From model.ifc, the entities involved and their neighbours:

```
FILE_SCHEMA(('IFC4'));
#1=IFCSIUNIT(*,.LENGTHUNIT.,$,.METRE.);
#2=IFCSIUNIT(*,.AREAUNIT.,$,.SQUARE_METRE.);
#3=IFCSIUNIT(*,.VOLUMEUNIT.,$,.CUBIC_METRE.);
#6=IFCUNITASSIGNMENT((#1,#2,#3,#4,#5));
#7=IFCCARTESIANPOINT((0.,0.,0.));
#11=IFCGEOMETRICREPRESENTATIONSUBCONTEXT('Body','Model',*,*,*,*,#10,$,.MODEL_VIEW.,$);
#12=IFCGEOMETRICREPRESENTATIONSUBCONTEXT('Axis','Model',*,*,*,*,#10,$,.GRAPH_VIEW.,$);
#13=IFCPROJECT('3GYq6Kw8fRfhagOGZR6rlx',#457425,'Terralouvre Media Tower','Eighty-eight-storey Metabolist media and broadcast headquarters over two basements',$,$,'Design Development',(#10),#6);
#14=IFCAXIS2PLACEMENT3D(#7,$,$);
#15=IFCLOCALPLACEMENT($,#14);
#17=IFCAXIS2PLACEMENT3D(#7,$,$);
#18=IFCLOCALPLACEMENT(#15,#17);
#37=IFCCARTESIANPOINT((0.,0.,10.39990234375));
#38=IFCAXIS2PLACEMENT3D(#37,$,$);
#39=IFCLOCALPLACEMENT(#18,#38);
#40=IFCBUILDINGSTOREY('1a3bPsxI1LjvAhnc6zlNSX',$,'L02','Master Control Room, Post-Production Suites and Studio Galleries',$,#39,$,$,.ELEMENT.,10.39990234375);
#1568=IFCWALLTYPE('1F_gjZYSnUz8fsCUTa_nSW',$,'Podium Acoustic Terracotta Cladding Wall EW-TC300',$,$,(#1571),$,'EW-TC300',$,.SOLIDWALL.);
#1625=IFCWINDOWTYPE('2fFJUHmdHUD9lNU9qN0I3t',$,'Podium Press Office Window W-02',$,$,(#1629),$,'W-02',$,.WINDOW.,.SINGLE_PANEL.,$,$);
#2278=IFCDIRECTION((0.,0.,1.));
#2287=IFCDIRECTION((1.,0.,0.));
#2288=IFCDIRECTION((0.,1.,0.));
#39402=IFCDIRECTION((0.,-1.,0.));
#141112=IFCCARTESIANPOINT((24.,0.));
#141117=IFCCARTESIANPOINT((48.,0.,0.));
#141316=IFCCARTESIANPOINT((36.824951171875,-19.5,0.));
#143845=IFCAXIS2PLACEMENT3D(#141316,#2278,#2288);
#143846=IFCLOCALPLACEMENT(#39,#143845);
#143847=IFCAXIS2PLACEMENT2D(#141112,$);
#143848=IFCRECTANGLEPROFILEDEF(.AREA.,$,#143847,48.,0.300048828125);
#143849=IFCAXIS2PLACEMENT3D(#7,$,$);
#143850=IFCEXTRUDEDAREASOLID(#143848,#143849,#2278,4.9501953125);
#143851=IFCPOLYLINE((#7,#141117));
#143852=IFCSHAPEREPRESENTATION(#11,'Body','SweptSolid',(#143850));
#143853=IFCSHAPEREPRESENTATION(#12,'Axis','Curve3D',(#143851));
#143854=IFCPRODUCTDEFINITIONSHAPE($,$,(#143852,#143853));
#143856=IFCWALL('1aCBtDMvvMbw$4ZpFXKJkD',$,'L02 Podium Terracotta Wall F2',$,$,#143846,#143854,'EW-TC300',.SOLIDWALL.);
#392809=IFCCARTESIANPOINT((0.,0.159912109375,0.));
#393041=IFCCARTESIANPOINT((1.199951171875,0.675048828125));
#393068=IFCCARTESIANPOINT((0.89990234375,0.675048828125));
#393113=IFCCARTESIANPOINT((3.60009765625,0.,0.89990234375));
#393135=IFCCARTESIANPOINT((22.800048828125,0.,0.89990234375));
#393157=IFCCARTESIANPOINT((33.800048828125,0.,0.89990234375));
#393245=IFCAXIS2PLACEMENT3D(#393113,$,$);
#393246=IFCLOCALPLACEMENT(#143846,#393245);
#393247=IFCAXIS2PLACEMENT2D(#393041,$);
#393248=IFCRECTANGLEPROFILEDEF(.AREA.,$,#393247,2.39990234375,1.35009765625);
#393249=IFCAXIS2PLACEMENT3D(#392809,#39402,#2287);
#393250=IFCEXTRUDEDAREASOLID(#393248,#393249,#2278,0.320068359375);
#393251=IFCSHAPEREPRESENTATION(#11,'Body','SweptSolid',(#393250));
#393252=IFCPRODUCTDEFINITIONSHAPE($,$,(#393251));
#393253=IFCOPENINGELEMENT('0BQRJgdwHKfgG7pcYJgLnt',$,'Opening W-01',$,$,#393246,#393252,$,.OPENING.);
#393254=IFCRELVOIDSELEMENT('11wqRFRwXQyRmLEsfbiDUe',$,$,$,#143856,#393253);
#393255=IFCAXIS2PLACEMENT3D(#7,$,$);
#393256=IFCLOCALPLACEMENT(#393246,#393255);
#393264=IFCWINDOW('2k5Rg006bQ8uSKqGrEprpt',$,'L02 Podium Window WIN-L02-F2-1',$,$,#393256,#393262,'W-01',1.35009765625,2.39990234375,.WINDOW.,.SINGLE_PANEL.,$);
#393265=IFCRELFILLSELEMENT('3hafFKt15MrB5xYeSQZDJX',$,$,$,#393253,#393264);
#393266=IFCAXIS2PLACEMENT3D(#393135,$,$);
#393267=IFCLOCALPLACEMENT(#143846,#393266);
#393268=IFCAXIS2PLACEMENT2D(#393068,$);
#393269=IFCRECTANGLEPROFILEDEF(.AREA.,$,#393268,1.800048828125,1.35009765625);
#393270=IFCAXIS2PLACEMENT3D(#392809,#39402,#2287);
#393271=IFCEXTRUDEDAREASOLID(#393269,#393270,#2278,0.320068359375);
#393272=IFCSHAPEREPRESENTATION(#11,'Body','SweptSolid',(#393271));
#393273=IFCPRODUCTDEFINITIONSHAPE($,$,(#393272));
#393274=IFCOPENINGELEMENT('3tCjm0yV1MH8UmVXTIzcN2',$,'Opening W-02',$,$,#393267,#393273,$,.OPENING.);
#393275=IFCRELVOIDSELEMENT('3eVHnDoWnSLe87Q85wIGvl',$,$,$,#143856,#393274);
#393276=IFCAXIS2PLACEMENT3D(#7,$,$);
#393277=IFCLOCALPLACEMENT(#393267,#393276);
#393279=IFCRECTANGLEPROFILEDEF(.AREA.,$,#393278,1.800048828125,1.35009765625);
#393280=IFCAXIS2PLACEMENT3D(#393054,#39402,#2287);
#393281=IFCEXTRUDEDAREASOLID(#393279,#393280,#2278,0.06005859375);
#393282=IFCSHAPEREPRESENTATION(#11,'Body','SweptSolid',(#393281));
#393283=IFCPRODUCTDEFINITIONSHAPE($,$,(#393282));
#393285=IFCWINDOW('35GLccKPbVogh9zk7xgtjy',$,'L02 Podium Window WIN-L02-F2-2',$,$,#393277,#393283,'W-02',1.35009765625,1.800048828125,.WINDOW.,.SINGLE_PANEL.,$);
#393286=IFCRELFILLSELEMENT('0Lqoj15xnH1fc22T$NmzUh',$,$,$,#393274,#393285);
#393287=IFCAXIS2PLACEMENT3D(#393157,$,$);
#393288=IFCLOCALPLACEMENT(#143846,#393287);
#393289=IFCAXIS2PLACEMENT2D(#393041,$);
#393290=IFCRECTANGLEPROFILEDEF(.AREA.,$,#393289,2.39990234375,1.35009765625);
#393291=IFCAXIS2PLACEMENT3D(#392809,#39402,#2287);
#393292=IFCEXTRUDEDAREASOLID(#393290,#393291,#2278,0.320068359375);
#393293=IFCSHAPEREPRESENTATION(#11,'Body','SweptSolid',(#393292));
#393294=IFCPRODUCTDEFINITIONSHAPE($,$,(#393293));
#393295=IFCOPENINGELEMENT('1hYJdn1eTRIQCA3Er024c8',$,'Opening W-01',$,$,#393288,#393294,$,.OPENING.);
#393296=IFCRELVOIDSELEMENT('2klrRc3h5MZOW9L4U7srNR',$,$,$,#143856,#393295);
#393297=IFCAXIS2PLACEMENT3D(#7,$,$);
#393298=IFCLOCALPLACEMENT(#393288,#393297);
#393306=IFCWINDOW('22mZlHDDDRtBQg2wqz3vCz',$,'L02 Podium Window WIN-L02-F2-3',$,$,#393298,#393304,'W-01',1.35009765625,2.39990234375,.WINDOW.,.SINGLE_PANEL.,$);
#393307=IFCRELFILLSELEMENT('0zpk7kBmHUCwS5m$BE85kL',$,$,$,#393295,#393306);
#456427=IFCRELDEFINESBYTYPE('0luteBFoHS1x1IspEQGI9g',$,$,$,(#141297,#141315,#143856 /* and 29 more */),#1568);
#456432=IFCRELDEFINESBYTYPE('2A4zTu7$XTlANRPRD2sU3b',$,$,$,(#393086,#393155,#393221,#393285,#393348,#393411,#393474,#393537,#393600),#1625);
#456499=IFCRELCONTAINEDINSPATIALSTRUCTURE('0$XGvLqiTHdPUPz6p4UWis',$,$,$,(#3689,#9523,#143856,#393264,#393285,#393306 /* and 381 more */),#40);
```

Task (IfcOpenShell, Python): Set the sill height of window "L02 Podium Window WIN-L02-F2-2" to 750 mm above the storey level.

```python
import numpy as np
import ifcopenshell
import ifcopenshell.api.geometry
import ifcopenshell.geom
import ifcopenshell.util.element
import ifcopenshell.util.placement
import ifcopenshell.util.shape
import ifcopenshell.util.unit

model = ifcopenshell.open("model.ifc")
unit_scale = ifcopenshell.util.unit.calculate_unit_scale(model)

window = model.by_id(393285)
opening = window.FillsVoids[0].RelatingOpeningElement
storey = ifcopenshell.util.element.get_container(window, ifc_class="IfcBuildingStorey")
level = ifcopenshell.util.placement.get_local_placement(storey.ObjectPlacement)[2, 3]

# The opening's origin need not be at the sill, so measure its lowest point.
shape = ifcopenshell.geom.create_shape(ifcopenshell.geom.settings(), opening)
bottom = ifcopenshell.util.shape.get_shape_bottom_elevation(shape, shape.geometry) / unit_scale
dz = level + 0.75 / unit_scale - bottom

shift = np.array([0.0, 0.0, dz])
# The window is placed relative to its opening, so it follows when the opening moves.
matrix = ifcopenshell.util.placement.get_local_placement(opening.ObjectPlacement)
matrix[:3, 3] += shift
ifcopenshell.api.geometry.edit_object_placement(
    model, product=opening, matrix=matrix, is_si=False, should_transform_children=True
)

print(f"moved by {dz * unit_scale:+.3f} m")

model.write("model-out.ifc")
```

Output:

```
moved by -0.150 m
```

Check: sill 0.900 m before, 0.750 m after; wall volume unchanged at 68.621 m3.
